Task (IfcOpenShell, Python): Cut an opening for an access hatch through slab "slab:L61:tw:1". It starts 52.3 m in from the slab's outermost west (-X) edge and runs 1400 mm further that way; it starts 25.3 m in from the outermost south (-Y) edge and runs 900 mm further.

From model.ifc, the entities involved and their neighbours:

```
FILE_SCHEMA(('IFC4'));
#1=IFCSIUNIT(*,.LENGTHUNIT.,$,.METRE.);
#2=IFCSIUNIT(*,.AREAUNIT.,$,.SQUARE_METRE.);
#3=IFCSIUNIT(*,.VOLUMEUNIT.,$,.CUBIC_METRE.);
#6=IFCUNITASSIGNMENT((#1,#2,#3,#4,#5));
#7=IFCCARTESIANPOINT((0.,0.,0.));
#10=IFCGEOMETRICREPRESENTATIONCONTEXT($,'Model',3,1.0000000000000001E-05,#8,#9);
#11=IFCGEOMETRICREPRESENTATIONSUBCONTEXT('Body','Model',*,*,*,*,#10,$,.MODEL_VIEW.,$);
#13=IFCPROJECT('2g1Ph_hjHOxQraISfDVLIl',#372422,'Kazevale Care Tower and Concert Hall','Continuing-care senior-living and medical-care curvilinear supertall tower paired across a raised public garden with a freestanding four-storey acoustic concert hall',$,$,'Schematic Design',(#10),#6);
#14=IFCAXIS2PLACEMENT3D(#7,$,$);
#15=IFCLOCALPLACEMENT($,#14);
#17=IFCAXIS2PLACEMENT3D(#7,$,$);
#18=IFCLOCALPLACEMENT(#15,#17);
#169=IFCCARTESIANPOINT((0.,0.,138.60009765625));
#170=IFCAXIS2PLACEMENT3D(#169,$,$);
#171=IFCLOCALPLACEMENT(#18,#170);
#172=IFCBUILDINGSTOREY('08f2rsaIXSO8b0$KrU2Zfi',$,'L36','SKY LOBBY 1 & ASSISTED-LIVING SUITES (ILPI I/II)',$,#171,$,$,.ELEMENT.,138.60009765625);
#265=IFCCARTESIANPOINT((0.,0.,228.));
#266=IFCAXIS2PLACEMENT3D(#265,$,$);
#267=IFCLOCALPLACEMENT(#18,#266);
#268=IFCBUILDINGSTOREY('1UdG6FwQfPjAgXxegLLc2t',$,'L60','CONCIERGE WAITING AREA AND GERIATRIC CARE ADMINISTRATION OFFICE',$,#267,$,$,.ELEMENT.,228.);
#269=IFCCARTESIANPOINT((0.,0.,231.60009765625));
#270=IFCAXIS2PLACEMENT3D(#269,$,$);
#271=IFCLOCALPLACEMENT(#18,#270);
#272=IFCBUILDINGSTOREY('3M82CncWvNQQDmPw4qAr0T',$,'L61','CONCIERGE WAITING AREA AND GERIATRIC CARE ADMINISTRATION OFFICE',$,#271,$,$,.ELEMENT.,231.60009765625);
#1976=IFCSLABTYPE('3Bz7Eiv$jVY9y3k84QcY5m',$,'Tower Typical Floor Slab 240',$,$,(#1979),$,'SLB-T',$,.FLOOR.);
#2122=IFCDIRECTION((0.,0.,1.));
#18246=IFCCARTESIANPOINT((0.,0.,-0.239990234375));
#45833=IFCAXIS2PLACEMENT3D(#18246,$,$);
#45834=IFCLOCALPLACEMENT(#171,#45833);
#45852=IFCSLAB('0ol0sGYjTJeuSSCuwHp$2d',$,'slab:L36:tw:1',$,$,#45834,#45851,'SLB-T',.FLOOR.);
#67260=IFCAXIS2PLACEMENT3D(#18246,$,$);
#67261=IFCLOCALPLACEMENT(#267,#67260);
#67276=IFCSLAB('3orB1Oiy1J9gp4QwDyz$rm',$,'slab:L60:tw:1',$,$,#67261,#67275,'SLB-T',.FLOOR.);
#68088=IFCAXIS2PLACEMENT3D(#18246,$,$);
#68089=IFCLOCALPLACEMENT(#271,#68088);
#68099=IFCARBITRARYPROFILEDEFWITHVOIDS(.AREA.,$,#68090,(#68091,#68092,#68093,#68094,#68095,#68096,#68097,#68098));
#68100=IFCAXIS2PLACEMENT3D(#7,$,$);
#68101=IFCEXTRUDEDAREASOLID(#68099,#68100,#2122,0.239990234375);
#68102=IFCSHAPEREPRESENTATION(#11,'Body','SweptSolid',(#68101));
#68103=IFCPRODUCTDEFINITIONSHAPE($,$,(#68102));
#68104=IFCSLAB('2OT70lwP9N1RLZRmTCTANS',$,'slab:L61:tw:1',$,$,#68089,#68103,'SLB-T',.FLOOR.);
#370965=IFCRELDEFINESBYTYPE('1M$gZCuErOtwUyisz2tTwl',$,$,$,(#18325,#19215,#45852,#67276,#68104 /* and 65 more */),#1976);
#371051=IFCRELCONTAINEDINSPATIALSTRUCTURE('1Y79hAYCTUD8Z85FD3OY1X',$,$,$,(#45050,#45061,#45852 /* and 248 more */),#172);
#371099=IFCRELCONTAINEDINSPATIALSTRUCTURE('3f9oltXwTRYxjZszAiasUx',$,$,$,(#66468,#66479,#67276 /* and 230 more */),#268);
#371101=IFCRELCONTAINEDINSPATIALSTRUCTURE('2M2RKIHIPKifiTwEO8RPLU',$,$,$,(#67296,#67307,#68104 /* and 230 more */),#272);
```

```python
import numpy as np
import ifcopenshell
import ifcopenshell.api.feature
import ifcopenshell.api.geometry
import ifcopenshell.api.root
import ifcopenshell.geom
import ifcopenshell.util.placement
import ifcopenshell.util.representation
import ifcopenshell.util.shape
import ifcopenshell.util.unit

model = ifcopenshell.open("model.ifc")
unit_scale = ifcopenshell.util.unit.calculate_unit_scale(model)
settings = ifcopenshell.geom.settings()


def volume(element):
    """Net volume in cubic metres, openings subtracted."""
    shape = ifcopenshell.geom.create_shape(settings, element)
    return ifcopenshell.util.shape.get_volume(shape.geometry)


slab = model.by_guid("2OT70lwP9N1RLZRmTCTANS")
before = volume(slab)

# Extent in the slab's own axes, in metres. The edges named are its -X and -Y sides.
slab_shape = ifcopenshell.geom.create_shape(settings, slab)
vertices = ifcopenshell.util.shape.get_vertices(slab_shape.geometry)
x_min, y_min, bottom = vertices.min(axis=0)
top = vertices[:, 2].max()

opening = ifcopenshell.api.root.create_entity(model, ifc_class="IfcOpeningElement", name="Access hatch opening", predefined_type="OPENING")
context = ifcopenshell.util.representation.get_context(model, "Model", "Body", "MODEL_VIEW")
width, depth = 1.4, 0.9
outline = [(0.0, 0.0), (width, 0.0), (width, depth), (0.0, depth), (0.0, 0.0)]
# Overshoot both faces by 50 mm so the cut is clean.
shape = ifcopenshell.api.geometry.add_slab_representation(
    model, context=context, depth=top - bottom + 0.1, polyline=outline
)
ifcopenshell.api.geometry.assign_representation(model, product=opening, representation=shape)

matrix = ifcopenshell.util.placement.get_local_placement(slab.ObjectPlacement)
matrix[:, 3] = matrix @ np.append(np.array([x_min + 52.3, y_min + 25.3, bottom - 0.05]) / unit_scale, 1.0)
ifcopenshell.api.geometry.edit_object_placement(model, product=opening, matrix=matrix, is_si=False)
ifcopenshell.api.feature.add_feature(model, feature=opening, element=slab)

after = volume(slab)

print(f"slab volume {before:.3f} -> {after:.3f} m3")

model.write("model-out.ifc")
```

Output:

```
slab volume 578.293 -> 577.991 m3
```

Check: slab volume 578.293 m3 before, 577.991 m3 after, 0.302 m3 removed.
